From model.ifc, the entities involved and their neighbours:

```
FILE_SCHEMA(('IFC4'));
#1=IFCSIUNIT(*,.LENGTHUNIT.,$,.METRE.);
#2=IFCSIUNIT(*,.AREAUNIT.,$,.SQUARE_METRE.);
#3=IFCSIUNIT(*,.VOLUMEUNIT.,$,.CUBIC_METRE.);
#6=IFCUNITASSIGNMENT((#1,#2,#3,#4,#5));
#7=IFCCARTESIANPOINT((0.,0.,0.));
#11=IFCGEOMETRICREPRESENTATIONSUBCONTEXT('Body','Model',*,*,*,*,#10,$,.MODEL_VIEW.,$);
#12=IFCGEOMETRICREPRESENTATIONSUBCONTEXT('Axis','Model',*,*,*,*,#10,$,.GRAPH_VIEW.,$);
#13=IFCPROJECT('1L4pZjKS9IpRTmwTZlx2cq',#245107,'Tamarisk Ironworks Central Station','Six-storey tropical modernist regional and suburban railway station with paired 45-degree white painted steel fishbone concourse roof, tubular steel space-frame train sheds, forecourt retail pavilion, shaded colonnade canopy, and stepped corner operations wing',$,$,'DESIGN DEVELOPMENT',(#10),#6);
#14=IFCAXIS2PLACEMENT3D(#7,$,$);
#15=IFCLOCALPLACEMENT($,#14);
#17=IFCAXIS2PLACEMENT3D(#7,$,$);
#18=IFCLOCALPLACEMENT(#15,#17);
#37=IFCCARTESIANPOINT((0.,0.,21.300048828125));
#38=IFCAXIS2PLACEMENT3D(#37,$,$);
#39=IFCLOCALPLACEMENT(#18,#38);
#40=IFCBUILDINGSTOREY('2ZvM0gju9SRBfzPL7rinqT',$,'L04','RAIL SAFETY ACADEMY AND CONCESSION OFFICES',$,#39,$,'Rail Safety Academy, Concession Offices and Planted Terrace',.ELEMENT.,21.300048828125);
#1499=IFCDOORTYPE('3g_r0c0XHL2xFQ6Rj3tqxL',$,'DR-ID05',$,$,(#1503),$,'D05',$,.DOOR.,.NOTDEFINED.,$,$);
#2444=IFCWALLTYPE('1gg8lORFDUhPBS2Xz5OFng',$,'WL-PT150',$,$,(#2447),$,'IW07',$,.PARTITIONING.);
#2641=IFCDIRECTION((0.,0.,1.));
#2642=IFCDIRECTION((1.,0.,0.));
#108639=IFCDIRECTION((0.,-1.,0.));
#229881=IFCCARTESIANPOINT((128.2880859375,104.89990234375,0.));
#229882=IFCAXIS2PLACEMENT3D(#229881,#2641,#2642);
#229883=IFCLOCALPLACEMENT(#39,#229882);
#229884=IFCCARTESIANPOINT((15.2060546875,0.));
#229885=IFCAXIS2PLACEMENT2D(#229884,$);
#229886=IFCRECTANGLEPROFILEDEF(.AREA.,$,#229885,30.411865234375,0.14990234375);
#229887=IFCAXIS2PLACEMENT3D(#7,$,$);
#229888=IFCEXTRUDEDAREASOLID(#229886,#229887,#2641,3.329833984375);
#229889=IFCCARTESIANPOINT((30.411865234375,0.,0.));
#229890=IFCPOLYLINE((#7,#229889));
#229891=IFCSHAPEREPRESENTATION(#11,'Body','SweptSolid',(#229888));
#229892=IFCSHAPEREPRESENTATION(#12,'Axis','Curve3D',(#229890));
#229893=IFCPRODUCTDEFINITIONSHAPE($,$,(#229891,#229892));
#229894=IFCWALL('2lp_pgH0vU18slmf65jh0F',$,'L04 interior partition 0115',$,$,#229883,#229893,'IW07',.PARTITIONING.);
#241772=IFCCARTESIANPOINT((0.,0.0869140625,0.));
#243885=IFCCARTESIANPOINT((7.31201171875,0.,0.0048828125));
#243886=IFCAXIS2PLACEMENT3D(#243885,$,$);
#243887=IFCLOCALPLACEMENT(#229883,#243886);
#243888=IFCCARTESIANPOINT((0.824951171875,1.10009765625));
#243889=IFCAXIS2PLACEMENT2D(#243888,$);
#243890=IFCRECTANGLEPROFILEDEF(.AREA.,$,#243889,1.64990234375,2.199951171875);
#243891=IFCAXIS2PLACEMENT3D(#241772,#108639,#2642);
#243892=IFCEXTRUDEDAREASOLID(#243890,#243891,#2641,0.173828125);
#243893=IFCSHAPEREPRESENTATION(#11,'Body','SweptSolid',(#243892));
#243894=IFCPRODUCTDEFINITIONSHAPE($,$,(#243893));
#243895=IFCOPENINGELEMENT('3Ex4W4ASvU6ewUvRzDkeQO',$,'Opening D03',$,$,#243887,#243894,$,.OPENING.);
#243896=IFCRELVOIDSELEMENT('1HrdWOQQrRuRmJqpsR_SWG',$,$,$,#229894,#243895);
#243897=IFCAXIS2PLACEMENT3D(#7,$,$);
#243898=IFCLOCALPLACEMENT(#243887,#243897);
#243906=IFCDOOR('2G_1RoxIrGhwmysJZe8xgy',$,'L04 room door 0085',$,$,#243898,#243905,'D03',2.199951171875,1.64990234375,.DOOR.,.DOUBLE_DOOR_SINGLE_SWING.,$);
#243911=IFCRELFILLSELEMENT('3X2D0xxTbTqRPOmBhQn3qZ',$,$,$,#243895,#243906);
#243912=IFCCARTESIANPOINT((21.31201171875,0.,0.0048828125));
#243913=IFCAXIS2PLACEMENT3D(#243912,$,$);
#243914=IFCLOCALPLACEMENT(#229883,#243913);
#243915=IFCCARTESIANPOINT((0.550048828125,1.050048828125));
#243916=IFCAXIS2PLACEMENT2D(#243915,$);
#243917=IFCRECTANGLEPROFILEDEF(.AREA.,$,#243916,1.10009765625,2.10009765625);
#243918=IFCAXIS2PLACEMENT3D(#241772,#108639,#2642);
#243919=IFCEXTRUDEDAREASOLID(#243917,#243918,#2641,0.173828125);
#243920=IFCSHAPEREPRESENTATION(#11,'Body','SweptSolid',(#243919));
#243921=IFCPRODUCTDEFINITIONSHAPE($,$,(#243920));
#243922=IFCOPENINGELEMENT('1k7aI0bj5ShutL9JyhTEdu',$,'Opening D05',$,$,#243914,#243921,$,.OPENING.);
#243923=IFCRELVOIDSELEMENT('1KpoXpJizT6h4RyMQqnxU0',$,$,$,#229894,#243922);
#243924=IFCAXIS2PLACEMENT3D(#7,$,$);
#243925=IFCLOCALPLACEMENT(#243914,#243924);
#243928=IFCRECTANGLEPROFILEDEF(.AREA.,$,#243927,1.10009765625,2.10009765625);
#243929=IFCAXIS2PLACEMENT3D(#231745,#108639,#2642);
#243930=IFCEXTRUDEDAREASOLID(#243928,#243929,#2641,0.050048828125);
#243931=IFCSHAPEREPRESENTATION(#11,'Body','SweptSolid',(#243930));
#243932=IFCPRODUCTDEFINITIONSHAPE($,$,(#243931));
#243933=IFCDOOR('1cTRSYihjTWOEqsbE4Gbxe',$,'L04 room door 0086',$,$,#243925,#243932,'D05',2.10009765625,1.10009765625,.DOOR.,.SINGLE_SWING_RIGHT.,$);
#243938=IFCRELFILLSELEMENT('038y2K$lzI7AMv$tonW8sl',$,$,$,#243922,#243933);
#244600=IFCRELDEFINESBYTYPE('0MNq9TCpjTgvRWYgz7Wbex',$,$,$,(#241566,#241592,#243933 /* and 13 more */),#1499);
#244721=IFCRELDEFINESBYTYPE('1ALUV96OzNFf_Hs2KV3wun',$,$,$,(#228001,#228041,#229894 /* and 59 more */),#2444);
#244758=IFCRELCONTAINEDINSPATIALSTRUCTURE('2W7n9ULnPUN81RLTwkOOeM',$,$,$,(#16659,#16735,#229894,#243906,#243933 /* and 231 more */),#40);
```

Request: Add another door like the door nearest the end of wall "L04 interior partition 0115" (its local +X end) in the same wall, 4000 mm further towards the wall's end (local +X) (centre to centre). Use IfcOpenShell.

```python
import ifcopenshell
import ifcopenshell.api.feature
import ifcopenshell.api.geometry
import ifcopenshell.api.root
import ifcopenshell.geom
import ifcopenshell.util.element
import ifcopenshell.util.placement
import ifcopenshell.util.shape

model = ifcopenshell.open("model.ifc")
settings = ifcopenshell.geom.settings()


def volume(element):
    """Net volume in cubic metres, openings subtracted."""
    shape = ifcopenshell.geom.create_shape(settings, element)
    return ifcopenshell.util.shape.get_volume(shape.geometry)


door = model.by_id(243933)
opening = door.FillsVoids[0].RelatingOpeningElement
wall = opening.VoidsElements[0].RelatingBuildingElement
before = volume(wall)
shift = ifcopenshell.util.placement.get_local_placement(wall.ObjectPlacement)[:3, 0] * 4.0

# copy_class copies the void relationship, type, container and properties, but no geometry.
new_opening = ifcopenshell.api.root.copy_class(model, product=opening)
new_opening.Representation = ifcopenshell.util.element.copy_deep(
    model, opening.Representation, exclude=["IfcGeometricRepresentationContext", "IfcRepresentationMap"]
)
new_door = ifcopenshell.api.root.copy_class(model, product=door)
new_door.Representation = ifcopenshell.util.element.copy_deep(
    model, door.Representation, exclude=["IfcGeometricRepresentationContext", "IfcRepresentationMap"]
)
new_door.Tag = None
ifcopenshell.api.feature.add_filling(model, opening=new_opening, element=new_door)

for old, new in ((opening, new_opening), (door, new_door)):
    matrix = ifcopenshell.util.placement.get_local_placement(old.ObjectPlacement)
    matrix[:3, 3] += shift
    ifcopenshell.api.geometry.edit_object_placement(model, product=new, matrix=matrix, is_si=False)

after = volume(wall)

print(f"wall volume {before:.3f} -> {after:.3f} m3")

model.write("model_rev.ifc")
```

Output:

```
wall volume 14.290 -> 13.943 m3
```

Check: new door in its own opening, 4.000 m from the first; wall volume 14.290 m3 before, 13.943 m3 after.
